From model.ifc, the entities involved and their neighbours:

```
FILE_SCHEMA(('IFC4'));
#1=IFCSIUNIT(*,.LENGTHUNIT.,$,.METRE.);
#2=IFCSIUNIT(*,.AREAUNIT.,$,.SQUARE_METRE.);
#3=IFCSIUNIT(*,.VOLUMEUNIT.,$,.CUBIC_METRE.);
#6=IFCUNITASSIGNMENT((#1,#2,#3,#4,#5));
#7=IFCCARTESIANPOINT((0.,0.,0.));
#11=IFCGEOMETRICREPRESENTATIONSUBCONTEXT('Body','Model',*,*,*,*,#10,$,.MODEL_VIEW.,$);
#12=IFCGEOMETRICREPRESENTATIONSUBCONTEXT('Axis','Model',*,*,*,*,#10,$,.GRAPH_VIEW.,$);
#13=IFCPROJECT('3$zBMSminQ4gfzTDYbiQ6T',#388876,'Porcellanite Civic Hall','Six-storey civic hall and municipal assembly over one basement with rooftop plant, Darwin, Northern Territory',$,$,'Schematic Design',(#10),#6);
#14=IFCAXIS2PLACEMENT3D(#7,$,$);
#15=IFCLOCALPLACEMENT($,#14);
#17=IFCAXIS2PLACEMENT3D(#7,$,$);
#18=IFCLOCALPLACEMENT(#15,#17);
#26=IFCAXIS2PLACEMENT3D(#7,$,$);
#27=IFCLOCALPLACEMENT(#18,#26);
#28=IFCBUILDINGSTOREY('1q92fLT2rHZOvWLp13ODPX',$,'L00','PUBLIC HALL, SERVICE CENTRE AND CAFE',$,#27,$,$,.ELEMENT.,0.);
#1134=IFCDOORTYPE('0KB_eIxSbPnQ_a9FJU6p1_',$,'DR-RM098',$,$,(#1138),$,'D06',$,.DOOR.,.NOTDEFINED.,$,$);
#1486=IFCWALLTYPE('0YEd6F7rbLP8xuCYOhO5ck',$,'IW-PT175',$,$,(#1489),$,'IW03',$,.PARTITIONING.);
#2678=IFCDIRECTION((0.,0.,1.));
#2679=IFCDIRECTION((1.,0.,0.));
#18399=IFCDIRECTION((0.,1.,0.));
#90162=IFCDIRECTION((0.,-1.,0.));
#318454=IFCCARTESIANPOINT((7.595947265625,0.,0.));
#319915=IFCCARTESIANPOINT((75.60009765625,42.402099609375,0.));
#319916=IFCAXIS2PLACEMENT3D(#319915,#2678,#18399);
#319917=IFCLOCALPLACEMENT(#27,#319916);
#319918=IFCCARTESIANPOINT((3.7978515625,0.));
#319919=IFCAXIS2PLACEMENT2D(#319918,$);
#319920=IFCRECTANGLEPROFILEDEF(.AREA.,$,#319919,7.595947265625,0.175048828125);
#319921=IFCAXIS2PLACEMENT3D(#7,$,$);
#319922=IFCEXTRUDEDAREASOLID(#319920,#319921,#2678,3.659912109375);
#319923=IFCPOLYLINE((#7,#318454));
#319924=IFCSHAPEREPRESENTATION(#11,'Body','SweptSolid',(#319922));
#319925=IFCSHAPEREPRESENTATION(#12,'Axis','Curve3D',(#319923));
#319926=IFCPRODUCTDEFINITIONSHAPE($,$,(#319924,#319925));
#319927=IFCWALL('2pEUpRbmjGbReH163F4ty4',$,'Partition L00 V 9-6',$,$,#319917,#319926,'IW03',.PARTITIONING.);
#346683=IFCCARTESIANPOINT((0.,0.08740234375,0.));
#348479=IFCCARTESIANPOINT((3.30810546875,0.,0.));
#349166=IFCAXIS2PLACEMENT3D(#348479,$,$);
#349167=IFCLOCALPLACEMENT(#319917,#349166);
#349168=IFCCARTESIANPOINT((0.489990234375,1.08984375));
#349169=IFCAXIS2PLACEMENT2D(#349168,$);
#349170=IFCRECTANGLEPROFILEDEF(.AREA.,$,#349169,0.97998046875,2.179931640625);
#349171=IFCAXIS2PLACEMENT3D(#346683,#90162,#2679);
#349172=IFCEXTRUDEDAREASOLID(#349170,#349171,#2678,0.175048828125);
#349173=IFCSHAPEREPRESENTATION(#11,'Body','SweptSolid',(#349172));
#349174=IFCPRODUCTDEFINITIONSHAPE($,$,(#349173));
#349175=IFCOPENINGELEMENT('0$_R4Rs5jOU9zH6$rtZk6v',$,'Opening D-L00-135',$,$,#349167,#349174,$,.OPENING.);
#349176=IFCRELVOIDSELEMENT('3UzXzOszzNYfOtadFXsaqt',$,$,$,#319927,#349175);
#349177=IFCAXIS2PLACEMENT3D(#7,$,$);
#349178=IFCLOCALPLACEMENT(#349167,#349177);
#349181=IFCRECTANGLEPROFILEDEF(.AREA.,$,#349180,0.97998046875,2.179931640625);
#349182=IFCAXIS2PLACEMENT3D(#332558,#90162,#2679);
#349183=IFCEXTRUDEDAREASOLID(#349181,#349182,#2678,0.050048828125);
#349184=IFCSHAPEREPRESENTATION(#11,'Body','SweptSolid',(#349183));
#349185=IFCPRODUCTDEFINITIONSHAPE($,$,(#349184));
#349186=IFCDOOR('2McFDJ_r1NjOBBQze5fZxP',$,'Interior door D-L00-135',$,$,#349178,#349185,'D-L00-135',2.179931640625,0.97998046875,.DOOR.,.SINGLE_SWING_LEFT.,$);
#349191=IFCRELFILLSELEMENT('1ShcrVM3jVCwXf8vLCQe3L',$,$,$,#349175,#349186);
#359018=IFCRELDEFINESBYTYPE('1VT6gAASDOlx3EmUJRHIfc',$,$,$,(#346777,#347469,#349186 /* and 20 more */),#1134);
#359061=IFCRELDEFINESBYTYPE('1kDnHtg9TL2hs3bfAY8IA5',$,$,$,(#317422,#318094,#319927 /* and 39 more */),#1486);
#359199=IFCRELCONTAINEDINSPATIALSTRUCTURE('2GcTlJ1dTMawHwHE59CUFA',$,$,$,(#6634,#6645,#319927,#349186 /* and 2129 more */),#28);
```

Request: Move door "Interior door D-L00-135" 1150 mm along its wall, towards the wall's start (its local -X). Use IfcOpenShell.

```python
import ifcopenshell
import ifcopenshell.api.geometry
import ifcopenshell.util.placement
import ifcopenshell.util.unit

model = ifcopenshell.open("model.ifc")
unit_scale = ifcopenshell.util.unit.calculate_unit_scale(model)

door = model.by_guid("2McFDJ_r1NjOBBQze5fZxP")
opening = door.FillsVoids[0].RelatingOpeningElement
wall = opening.VoidsElements[0].RelatingBuildingElement

wall_matrix = ifcopenshell.util.placement.get_local_placement(wall.ObjectPlacement)
shift = wall_matrix[:3, 0] * -1.15 / unit_scale
before = ifcopenshell.util.placement.get_local_placement(door.ObjectPlacement)[:3, 3].copy()

# The door is placed relative to its opening, so it follows when the opening moves.
matrix = ifcopenshell.util.placement.get_local_placement(opening.ObjectPlacement)
matrix[:3, 3] += shift
ifcopenshell.api.geometry.edit_object_placement(
    model, product=opening, matrix=matrix, is_si=False, should_transform_children=True
)

after = ifcopenshell.util.placement.get_local_placement(door.ObjectPlacement)[:3, 3]
print("door moved by", (after - before).round(3) + 0.0)

model.write("model_edited.ifc")
```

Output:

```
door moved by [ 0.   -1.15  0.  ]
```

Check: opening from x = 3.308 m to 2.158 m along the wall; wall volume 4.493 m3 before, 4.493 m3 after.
